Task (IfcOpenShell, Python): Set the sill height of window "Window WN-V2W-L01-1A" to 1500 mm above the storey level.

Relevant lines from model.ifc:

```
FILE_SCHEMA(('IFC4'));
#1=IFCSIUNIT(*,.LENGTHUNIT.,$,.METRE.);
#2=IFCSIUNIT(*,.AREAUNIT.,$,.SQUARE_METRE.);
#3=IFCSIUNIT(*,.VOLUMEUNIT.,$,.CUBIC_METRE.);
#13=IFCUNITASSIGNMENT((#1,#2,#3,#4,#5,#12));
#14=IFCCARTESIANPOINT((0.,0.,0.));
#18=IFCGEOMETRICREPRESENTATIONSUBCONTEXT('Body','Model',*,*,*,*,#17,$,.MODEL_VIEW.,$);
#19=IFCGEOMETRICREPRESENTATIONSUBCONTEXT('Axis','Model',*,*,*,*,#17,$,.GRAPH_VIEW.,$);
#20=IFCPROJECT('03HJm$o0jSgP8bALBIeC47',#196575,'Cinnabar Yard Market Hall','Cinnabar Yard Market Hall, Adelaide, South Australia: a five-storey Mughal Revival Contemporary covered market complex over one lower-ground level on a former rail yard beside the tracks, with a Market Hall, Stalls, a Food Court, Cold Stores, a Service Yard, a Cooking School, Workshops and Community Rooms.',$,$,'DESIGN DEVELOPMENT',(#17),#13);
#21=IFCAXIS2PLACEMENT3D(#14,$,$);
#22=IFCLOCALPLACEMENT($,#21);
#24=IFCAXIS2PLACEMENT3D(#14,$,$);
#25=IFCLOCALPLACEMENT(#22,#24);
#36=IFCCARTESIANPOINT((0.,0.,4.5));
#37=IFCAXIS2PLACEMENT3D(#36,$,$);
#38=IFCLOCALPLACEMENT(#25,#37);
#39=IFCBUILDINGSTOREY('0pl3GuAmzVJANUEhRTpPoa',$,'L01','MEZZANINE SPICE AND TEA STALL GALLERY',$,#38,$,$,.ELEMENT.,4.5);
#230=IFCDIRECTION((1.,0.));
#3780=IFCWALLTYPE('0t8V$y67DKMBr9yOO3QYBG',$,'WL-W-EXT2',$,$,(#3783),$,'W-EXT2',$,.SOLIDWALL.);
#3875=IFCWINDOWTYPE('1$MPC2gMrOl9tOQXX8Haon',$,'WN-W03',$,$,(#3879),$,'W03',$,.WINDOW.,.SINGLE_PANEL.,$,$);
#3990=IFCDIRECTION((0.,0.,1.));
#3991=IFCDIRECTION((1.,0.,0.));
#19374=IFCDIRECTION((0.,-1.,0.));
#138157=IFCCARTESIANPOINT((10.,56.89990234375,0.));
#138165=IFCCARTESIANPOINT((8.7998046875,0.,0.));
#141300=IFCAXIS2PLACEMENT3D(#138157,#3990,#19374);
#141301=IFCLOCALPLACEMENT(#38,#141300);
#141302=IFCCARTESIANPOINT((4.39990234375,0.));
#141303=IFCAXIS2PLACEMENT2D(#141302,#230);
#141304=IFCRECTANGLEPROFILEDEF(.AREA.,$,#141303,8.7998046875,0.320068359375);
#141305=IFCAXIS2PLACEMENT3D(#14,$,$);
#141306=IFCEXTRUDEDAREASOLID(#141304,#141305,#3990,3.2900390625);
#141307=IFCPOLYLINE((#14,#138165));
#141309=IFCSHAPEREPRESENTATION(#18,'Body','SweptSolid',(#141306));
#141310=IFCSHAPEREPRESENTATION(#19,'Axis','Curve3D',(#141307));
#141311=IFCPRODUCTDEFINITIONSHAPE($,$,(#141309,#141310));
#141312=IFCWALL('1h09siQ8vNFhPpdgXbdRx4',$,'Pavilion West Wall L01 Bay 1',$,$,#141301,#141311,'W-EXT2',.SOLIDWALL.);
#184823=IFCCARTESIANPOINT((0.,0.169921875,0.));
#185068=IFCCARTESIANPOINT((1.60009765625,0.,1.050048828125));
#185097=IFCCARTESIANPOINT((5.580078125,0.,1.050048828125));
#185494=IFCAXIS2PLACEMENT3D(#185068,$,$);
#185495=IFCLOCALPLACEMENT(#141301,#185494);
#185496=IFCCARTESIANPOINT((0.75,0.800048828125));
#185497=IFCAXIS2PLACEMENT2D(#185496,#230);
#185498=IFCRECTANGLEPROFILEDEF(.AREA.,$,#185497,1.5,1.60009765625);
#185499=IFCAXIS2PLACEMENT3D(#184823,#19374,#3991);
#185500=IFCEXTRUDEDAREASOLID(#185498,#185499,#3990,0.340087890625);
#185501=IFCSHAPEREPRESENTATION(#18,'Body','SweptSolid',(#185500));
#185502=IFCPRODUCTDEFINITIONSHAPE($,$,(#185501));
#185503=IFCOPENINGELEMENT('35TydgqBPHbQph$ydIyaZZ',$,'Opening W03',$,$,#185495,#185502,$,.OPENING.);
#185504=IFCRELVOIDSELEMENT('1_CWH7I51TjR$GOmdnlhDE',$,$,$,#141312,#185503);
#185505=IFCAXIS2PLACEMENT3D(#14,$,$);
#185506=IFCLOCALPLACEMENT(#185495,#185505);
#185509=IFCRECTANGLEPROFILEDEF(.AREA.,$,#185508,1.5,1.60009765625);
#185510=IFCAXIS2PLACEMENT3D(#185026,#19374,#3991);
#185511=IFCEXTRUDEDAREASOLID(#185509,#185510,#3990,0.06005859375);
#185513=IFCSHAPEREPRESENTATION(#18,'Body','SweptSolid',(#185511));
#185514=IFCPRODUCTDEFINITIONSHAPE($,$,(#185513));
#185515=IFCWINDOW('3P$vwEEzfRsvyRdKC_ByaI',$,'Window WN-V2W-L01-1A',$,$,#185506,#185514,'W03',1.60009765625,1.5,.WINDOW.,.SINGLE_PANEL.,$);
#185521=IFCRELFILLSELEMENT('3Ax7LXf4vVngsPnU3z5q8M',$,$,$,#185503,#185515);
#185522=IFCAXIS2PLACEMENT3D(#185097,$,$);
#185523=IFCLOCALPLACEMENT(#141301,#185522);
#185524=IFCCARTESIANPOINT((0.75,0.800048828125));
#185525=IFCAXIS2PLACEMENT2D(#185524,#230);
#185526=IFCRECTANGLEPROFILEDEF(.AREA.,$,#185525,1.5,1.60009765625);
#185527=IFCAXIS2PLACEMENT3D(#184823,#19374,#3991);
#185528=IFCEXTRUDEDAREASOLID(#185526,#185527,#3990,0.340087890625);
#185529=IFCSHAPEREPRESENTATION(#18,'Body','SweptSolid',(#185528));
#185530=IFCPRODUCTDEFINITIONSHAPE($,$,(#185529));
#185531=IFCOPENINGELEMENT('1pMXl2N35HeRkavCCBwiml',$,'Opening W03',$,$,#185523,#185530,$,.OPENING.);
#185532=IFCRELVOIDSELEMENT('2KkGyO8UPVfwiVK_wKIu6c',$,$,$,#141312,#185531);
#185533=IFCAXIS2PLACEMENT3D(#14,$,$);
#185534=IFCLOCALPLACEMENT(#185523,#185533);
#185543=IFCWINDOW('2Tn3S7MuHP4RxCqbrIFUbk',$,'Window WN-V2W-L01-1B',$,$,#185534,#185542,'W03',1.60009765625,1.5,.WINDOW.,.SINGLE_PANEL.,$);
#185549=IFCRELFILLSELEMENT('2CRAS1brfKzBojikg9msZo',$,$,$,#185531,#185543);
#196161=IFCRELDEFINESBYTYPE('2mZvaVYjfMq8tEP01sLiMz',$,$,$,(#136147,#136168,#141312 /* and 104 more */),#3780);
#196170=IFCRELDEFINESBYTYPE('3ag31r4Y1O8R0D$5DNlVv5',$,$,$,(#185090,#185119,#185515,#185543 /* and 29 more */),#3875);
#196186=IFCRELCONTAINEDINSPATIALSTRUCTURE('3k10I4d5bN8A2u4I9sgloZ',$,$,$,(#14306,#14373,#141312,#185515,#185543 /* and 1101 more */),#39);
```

```python
import numpy as np
import ifcopenshell
import ifcopenshell.api.geometry
import ifcopenshell.geom
import ifcopenshell.util.element
import ifcopenshell.util.placement
import ifcopenshell.util.shape
import ifcopenshell.util.unit

model = ifcopenshell.open("model.ifc")
unit_scale = ifcopenshell.util.unit.calculate_unit_scale(model)

window = model.by_guid("3P$vwEEzfRsvyRdKC_ByaI")
opening = window.FillsVoids[0].RelatingOpeningElement
storey = ifcopenshell.util.element.get_container(window, ifc_class="IfcBuildingStorey")
level = ifcopenshell.util.placement.get_local_placement(storey.ObjectPlacement)[2, 3]

# The opening's origin need not be at the sill, so measure its lowest point.
shape = ifcopenshell.geom.create_shape(ifcopenshell.geom.settings(), opening)
bottom = ifcopenshell.util.shape.get_shape_bottom_elevation(shape, shape.geometry) / unit_scale
dz = level + 1.5 - bottom

shift = np.array([0.0, 0.0, dz])
# The window is placed relative to its opening, so it follows when the opening moves.
matrix = ifcopenshell.util.placement.get_local_placement(opening.ObjectPlacement)
matrix[:3, 3] += shift
ifcopenshell.api.geometry.edit_object_placement(
    model, product=opening, matrix=matrix, is_si=False, should_transform_children=True
)

print(f"moved by {dz * unit_scale:+.3f} m")

model.write("model_rev.ifc")
```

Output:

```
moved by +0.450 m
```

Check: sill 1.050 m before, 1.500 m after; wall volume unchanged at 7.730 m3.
